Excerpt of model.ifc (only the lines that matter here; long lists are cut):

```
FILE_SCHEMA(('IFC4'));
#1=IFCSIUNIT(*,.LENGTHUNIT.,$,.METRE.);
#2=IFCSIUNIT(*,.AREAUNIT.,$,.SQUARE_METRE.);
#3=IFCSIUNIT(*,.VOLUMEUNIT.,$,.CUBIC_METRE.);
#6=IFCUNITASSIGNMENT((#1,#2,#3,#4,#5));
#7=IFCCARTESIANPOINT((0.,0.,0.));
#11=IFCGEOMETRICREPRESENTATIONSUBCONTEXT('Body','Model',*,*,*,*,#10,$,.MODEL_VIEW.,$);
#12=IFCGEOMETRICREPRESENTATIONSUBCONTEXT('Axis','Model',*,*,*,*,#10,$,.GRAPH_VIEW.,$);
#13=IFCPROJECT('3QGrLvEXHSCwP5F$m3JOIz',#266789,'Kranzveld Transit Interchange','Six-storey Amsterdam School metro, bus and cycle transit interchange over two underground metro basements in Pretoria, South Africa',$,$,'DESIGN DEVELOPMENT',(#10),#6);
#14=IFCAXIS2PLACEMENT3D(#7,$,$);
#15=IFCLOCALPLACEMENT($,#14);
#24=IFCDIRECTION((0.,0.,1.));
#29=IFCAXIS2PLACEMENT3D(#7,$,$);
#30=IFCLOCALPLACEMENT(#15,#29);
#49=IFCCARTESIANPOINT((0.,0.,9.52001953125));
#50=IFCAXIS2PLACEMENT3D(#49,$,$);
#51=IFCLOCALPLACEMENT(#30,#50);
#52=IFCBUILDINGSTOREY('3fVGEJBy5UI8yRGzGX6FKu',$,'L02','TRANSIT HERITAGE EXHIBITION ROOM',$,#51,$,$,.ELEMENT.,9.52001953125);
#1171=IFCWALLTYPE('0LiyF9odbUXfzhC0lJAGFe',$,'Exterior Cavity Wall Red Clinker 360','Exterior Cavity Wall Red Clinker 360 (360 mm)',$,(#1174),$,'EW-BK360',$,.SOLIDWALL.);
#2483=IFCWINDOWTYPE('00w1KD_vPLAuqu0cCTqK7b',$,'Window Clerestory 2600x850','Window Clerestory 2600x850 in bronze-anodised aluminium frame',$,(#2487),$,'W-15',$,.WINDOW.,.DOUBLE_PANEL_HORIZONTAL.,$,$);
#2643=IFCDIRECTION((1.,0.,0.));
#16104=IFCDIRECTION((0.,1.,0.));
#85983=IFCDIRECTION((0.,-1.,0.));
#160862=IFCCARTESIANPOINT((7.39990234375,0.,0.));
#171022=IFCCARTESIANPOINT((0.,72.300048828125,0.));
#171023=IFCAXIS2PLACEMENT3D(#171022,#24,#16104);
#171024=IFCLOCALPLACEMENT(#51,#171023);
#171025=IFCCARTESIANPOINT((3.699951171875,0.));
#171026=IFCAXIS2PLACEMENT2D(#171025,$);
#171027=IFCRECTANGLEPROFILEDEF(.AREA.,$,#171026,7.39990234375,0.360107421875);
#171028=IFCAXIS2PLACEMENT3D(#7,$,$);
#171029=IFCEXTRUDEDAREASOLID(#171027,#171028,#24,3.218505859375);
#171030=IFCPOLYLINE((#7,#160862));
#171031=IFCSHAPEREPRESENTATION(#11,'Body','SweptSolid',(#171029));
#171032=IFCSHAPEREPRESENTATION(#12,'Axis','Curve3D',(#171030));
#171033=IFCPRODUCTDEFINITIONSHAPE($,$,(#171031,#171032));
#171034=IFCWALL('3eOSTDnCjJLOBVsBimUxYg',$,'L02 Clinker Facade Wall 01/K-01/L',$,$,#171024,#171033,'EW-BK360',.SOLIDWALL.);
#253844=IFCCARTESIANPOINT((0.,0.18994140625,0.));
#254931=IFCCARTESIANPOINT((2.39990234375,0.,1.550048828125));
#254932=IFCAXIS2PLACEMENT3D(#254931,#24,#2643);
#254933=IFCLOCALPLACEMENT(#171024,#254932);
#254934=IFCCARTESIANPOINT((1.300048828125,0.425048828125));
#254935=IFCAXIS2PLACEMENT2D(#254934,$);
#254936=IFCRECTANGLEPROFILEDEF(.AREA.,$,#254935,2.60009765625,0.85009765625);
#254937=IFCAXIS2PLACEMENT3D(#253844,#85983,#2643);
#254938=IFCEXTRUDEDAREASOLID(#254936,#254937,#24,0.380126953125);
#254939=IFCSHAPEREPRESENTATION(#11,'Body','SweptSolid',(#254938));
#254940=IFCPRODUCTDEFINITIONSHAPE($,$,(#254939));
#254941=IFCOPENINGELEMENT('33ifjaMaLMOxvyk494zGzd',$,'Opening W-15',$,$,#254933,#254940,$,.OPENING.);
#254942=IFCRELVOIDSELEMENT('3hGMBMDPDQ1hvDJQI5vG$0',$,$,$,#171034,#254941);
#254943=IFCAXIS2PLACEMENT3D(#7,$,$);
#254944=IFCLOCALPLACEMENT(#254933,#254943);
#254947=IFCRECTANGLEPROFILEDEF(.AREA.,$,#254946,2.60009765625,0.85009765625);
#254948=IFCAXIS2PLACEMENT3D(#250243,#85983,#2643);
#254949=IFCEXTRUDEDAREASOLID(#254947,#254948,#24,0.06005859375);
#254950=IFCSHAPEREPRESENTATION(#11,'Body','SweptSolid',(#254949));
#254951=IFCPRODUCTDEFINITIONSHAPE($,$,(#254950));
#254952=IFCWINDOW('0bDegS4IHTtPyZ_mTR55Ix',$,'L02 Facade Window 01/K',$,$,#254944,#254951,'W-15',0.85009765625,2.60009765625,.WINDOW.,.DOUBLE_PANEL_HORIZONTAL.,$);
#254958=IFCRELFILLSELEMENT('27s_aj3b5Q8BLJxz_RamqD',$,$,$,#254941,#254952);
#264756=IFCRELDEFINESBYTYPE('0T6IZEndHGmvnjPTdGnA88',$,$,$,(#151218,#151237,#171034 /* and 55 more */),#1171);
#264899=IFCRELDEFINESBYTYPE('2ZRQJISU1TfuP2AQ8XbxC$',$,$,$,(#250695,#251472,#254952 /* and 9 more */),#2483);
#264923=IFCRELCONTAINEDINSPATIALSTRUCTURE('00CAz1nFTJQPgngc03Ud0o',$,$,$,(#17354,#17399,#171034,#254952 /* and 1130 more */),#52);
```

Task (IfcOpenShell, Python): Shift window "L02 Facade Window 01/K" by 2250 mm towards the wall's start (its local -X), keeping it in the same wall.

```python
import ifcopenshell
import ifcopenshell.api.geometry
import ifcopenshell.util.placement

model = ifcopenshell.open("model.ifc")

window = model.by_guid("0bDegS4IHTtPyZ_mTR55Ix")
opening = window.FillsVoids[0].RelatingOpeningElement
wall = opening.VoidsElements[0].RelatingBuildingElement

wall_matrix = ifcopenshell.util.placement.get_local_placement(wall.ObjectPlacement)
shift = wall_matrix[:3, 0] * -2.25
before = ifcopenshell.util.placement.get_local_placement(window.ObjectPlacement)[:3, 3].copy()

# The window is placed relative to its opening, so it follows when the opening moves.
matrix = ifcopenshell.util.placement.get_local_placement(opening.ObjectPlacement)
matrix[:3, 3] += shift
ifcopenshell.api.geometry.edit_object_placement(
    model, product=opening, matrix=matrix, is_si=False, should_transform_children=True
)

after = ifcopenshell.util.placement.get_local_placement(window.ObjectPlacement)[:3, 3]
print("window moved by", (after - before).round(3) + 0.0)

model.write("model_updated.ifc")
```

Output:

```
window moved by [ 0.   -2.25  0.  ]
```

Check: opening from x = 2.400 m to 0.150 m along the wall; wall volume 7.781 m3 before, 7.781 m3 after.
